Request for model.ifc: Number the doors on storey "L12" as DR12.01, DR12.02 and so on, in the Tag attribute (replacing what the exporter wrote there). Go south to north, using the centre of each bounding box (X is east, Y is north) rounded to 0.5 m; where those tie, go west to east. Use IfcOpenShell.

First a look at what the model holds.

```python
import ifcopenshell
import ifcopenshell.util.element
import ifcopenshell.util.placement

model = ifcopenshell.open("model.ifc")
print(model.schema)
storey = next(s for s in model.by_type("IfcBuildingStorey") if s.Name == "L12")
doors = [e for e in ifcopenshell.util.element.get_decomposition(storey) if e.is_a("IfcDoor")]
for e in sorted(doors, key=lambda e: e.id()):
    origin = ifcopenshell.util.placement.get_local_placement(e.ObjectPlacement)[:3, 3]
    print(e.id(), e.Tag, e.Name, origin.round(2) + 0.0, sep=" | ")
```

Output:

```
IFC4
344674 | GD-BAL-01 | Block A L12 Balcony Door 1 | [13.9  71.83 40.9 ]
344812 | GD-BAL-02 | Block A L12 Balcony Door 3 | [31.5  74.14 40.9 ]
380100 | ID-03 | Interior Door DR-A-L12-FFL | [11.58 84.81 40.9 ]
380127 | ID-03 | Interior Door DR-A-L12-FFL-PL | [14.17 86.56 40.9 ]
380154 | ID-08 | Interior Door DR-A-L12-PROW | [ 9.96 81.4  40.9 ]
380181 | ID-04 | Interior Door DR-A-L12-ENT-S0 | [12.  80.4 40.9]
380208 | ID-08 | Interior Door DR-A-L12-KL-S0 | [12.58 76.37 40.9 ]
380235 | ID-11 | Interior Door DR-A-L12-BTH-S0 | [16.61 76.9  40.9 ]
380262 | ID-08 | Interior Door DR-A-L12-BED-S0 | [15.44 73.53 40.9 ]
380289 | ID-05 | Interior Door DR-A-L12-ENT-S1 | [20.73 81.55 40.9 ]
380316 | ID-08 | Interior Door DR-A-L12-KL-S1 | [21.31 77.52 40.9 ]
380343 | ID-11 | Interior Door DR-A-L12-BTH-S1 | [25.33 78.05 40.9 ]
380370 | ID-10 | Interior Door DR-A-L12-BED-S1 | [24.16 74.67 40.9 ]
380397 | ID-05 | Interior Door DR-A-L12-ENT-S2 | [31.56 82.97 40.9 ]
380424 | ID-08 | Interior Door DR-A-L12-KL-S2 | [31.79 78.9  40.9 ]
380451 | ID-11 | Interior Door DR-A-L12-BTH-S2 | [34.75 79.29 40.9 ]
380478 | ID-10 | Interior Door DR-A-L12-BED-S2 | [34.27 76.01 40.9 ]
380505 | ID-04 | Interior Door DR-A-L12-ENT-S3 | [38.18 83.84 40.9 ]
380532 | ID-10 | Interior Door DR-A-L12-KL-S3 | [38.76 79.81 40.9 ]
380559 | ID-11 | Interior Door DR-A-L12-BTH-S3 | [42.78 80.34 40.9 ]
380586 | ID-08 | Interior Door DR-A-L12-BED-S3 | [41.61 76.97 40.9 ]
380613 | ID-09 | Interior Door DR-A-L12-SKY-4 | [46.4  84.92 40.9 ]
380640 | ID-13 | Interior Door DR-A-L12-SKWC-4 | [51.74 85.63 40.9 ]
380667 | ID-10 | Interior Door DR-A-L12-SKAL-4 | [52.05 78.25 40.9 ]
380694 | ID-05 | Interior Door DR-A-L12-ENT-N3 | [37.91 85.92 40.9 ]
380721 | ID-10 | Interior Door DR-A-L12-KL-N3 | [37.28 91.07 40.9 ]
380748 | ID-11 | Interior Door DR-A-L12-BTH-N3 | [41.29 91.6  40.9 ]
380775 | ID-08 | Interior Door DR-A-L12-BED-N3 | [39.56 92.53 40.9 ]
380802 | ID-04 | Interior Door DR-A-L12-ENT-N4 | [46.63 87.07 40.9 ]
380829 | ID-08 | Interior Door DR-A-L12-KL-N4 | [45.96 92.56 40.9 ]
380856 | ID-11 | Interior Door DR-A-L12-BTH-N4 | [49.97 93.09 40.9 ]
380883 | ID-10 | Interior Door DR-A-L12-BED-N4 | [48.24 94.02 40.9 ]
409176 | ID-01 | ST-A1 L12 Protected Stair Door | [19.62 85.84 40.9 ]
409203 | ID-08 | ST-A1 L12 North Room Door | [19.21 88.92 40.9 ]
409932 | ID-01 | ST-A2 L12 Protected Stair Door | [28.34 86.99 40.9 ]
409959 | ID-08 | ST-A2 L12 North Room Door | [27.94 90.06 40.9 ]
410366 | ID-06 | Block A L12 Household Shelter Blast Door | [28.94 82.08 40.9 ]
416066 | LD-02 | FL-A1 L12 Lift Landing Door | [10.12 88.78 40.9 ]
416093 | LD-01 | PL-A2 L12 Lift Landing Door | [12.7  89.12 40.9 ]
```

```python
import ifcopenshell
import ifcopenshell.geom
import ifcopenshell.util.element
import ifcopenshell.util.shape

model = ifcopenshell.open("model.ifc")
settings = ifcopenshell.geom.settings()
settings.set("use-world-coords", True)


def centre(element):
    shape = ifcopenshell.geom.create_shape(settings, element)
    return ifcopenshell.util.shape.get_bbox_centroid(shape.geometry)


storey = next(s for s in model.by_type("IfcBuildingStorey") if s.Name == "L12")
doors = [e for e in ifcopenshell.util.element.get_decomposition(storey) if e.is_a("IfcDoor")]

# Insertion points can sit at a corner or the storey origin, so sort by the geometry (in metres).
centres = {e: centre(e) for e in doors}
doors.sort(key=lambda e: (round(centres[e][1] / 0.5), centres[e][0]))

for i, e in enumerate(doors, start=1):
    number = f"DR12.{i:02d}"
    e.Tag = number
    print(e.id(), number)

model.write("model_rev.ifc")
```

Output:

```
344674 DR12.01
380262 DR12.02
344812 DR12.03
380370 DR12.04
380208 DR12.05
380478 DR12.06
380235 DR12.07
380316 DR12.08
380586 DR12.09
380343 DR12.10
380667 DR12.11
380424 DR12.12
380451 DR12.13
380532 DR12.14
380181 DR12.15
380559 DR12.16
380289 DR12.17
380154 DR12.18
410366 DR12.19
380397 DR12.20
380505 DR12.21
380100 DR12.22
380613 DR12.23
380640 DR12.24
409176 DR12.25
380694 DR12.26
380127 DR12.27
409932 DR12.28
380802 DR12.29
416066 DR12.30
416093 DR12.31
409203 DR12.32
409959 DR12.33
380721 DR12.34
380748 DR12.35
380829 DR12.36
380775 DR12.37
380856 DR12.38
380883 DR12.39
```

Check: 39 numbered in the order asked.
